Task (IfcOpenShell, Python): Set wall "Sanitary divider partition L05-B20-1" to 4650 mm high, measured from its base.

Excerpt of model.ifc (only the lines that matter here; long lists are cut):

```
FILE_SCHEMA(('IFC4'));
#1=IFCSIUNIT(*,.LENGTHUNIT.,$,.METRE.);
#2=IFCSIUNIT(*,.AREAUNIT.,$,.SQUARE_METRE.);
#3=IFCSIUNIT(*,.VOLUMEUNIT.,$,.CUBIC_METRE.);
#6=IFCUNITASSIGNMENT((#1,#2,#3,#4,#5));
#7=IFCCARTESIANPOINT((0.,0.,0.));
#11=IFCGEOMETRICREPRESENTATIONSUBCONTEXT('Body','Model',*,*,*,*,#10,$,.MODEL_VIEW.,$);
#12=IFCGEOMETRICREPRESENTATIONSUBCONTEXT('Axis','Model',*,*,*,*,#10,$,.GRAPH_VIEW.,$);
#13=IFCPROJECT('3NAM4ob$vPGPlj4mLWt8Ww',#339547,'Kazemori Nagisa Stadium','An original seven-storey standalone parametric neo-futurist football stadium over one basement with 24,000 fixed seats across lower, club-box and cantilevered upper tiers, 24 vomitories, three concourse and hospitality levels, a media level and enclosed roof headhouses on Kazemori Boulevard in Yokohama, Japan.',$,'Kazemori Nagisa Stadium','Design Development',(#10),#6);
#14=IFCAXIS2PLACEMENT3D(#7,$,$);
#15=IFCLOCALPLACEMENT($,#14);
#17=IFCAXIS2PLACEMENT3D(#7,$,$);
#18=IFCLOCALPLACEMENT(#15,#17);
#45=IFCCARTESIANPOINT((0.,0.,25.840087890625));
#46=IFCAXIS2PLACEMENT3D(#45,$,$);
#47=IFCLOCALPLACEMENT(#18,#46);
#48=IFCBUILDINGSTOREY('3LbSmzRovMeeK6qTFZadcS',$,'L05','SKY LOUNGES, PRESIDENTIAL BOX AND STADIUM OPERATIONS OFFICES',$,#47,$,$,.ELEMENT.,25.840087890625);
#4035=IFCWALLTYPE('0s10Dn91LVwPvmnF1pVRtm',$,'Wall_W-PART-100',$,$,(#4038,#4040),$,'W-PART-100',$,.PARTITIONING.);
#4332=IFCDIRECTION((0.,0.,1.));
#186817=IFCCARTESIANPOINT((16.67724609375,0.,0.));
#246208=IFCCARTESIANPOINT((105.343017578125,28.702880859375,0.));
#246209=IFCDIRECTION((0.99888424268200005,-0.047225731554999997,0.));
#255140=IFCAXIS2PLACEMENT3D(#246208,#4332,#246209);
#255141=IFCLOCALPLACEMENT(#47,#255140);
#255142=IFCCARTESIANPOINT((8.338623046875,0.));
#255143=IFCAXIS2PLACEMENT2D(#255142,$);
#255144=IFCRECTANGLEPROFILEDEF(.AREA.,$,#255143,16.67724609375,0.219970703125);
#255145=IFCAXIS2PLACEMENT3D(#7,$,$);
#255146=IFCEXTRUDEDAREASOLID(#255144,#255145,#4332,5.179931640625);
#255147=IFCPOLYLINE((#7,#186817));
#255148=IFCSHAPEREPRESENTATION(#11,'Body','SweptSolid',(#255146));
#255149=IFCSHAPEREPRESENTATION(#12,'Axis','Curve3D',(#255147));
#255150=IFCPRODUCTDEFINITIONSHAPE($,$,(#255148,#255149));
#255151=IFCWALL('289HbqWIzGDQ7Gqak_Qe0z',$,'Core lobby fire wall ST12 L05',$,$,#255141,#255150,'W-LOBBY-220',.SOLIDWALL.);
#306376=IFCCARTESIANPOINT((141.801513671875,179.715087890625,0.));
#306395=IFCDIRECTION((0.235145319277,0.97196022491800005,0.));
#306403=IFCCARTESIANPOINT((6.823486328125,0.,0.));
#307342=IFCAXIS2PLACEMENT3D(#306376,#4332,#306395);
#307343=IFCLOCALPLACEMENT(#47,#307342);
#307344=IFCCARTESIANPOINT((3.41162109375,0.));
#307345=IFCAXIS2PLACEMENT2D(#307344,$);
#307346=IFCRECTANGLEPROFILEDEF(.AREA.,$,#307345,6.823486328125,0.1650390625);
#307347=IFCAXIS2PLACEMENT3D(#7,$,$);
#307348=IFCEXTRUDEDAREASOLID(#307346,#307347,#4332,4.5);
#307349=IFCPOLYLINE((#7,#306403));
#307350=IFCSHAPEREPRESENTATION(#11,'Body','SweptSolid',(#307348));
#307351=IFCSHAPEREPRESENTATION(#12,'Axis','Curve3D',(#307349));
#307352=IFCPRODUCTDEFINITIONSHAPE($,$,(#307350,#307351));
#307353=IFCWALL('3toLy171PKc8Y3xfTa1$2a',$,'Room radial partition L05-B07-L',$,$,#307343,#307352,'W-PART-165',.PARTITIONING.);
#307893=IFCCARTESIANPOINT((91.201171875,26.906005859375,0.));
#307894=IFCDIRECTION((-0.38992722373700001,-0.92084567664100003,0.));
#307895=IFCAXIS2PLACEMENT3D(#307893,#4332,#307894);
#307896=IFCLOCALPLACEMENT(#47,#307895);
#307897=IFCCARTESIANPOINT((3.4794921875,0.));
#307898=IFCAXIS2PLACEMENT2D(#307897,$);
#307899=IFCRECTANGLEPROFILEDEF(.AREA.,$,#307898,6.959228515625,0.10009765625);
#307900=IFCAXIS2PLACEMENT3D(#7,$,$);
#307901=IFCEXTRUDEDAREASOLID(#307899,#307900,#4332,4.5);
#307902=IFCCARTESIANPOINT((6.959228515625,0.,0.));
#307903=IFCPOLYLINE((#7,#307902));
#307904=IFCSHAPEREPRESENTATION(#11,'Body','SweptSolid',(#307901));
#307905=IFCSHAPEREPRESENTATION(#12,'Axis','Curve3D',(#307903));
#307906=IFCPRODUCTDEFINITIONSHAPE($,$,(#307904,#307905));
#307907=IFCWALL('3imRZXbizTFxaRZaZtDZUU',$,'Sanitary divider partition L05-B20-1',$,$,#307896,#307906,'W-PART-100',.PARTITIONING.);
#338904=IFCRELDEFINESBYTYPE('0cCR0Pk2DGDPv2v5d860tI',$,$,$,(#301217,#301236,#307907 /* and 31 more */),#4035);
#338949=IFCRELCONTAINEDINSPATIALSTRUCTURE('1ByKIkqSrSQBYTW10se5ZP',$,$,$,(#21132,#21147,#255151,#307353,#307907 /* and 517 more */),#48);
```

```python
import ifcopenshell
import ifcopenshell.geom
import ifcopenshell.util.representation
import ifcopenshell.util.shape
import ifcopenshell.util.unit

model = ifcopenshell.open("model.ifc")
unit_scale = ifcopenshell.util.unit.calculate_unit_scale(model)
settings = ifcopenshell.geom.settings()


def volume(element):
    """Net volume in cubic metres, openings subtracted."""
    shape = ifcopenshell.geom.create_shape(settings, element)
    return ifcopenshell.util.shape.get_volume(shape.geometry)


wall = model.by_guid("3imRZXbizTFxaRZaZtDZUU")
before = volume(wall)

body = ifcopenshell.util.representation.get_representation(wall, "Model", "Body")
solid = body.Items[0]
old_height = solid.Depth
solid.Depth = 4.65 / unit_scale
after = volume(wall)

print(f"height {old_height:g} -> {solid.Depth:g}, volume {before:.3f} -> {after:.3f} m3")

model.write("model_edited.ifc")
```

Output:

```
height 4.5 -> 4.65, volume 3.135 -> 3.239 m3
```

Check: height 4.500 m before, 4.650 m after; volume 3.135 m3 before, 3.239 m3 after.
